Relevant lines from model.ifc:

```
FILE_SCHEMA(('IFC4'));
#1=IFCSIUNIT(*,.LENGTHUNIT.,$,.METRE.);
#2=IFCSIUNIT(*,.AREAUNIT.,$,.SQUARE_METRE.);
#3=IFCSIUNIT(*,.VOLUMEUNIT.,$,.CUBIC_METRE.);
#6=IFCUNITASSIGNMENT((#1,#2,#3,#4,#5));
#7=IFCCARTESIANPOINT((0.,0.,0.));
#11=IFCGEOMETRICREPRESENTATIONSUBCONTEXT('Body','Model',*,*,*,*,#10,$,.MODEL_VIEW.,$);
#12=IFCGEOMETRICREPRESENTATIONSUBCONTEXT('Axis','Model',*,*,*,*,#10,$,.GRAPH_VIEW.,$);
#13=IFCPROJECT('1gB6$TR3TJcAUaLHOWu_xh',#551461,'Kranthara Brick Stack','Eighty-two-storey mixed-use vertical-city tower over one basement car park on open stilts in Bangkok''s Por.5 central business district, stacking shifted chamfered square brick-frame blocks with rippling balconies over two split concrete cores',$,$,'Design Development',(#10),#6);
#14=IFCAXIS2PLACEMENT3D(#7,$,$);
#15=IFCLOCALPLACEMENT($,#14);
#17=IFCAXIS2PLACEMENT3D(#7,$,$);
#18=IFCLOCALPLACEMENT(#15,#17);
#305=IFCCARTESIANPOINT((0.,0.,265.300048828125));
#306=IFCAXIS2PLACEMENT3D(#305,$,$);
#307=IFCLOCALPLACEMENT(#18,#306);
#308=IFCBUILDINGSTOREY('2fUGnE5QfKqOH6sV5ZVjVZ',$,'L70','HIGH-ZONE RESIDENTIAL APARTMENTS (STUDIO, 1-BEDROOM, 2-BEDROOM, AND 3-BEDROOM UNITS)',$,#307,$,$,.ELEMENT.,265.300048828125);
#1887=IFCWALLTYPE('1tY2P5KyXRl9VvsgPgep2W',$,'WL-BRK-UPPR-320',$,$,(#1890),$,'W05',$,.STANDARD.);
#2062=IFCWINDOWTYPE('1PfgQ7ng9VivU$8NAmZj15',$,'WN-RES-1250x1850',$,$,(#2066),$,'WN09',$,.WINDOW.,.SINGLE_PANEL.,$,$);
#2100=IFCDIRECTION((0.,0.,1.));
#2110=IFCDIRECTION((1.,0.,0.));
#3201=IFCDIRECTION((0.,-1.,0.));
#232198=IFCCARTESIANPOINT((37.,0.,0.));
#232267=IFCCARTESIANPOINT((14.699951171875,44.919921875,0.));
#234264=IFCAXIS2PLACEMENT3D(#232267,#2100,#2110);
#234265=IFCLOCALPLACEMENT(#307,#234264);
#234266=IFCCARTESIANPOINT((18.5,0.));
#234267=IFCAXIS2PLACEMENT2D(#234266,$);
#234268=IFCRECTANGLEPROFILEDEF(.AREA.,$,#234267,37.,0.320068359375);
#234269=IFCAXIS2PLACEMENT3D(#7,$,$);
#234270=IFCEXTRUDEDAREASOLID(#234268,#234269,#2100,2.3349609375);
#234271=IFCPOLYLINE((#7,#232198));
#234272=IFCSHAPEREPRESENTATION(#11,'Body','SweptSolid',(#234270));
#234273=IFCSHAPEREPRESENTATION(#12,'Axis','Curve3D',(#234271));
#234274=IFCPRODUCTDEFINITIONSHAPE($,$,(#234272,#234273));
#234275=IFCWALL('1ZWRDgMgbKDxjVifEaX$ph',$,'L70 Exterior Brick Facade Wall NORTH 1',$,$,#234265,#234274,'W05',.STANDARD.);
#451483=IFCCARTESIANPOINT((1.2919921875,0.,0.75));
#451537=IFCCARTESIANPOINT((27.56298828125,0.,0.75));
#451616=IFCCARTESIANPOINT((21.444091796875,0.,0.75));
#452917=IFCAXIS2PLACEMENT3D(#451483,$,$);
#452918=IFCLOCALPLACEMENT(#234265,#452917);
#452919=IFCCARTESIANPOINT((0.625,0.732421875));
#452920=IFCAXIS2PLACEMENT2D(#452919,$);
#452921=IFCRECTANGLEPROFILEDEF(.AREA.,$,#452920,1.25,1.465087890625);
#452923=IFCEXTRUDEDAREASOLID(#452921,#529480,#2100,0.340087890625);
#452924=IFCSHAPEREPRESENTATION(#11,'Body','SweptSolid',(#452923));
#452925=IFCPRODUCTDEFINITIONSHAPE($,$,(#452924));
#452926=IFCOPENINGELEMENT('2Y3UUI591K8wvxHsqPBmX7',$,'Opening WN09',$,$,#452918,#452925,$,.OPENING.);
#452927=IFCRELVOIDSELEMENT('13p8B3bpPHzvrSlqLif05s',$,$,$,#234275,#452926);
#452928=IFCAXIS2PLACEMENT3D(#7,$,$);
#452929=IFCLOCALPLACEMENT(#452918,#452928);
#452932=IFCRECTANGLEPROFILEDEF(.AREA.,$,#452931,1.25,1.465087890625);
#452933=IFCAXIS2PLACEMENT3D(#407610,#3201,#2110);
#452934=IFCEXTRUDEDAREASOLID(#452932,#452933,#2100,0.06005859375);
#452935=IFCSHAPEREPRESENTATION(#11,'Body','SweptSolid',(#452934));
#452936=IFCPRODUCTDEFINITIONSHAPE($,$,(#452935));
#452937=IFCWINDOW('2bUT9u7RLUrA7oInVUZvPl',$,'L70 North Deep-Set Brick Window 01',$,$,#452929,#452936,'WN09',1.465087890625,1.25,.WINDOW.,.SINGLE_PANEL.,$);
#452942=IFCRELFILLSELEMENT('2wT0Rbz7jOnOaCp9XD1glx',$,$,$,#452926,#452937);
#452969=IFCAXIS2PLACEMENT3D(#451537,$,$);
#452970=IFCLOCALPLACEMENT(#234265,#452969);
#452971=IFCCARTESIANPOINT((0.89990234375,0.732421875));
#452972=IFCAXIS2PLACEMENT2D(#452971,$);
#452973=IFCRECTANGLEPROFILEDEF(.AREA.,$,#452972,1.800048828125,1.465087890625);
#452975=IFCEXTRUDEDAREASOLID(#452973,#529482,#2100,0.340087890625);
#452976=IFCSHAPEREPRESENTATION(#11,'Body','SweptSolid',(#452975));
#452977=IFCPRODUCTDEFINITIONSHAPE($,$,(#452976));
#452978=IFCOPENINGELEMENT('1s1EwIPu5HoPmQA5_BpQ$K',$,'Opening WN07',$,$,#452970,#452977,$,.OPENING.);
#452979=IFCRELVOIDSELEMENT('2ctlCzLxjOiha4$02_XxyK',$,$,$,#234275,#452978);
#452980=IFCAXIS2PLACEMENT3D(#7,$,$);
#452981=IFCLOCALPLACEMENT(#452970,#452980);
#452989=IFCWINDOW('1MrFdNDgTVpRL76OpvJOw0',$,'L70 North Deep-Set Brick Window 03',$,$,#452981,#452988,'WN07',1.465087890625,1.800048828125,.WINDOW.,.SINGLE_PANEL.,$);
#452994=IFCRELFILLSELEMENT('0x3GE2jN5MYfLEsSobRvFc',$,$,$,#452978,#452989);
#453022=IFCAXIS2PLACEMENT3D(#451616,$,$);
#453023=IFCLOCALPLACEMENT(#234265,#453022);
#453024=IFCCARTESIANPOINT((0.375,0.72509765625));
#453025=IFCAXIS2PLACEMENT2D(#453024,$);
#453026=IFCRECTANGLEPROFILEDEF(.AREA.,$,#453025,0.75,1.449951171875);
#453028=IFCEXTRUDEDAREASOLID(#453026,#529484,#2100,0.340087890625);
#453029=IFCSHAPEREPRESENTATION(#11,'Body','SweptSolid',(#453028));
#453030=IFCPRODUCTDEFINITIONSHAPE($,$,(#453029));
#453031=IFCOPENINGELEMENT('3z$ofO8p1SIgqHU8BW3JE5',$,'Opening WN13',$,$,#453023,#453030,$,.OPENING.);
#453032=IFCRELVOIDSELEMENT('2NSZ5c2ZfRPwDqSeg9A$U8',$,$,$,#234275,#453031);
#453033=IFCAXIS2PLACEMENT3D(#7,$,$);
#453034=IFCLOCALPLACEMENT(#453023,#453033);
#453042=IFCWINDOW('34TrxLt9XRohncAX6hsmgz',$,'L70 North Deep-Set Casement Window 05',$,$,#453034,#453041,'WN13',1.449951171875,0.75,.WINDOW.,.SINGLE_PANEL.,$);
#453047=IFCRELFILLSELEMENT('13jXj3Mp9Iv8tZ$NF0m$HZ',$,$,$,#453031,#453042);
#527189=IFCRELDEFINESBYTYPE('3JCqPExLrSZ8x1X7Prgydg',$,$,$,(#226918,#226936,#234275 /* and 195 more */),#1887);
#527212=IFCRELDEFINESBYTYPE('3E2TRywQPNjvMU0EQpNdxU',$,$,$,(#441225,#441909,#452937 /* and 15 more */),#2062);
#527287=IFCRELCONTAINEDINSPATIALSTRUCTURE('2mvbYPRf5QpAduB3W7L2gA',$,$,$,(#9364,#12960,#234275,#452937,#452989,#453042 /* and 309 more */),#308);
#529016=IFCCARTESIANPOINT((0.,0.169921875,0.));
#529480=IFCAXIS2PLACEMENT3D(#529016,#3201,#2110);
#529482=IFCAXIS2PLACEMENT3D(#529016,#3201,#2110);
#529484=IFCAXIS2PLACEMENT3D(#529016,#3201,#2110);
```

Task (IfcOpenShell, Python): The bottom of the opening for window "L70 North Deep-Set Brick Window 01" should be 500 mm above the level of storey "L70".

```python
import numpy as np
import ifcopenshell
import ifcopenshell.api.geometry
import ifcopenshell.geom
import ifcopenshell.util.element
import ifcopenshell.util.placement
import ifcopenshell.util.shape
import ifcopenshell.util.unit

model = ifcopenshell.open("model.ifc")
unit_scale = ifcopenshell.util.unit.calculate_unit_scale(model)

window = model.by_guid("2bUT9u7RLUrA7oInVUZvPl")
opening = window.FillsVoids[0].RelatingOpeningElement
storey = ifcopenshell.util.element.get_container(window, ifc_class="IfcBuildingStorey")
level = ifcopenshell.util.placement.get_local_placement(storey.ObjectPlacement)[2, 3]

# The opening's origin need not be at the sill, so measure its lowest point.
shape = ifcopenshell.geom.create_shape(ifcopenshell.geom.settings(), opening)
bottom = ifcopenshell.util.shape.get_shape_bottom_elevation(shape, shape.geometry) / unit_scale
dz = level + 0.5 - bottom

shift = np.array([0.0, 0.0, dz])
# The window is placed relative to its opening, so it follows when the opening moves.
matrix = ifcopenshell.util.placement.get_local_placement(opening.ObjectPlacement)
matrix[:3, 3] += shift
ifcopenshell.api.geometry.edit_object_placement(
    model, product=opening, matrix=matrix, is_si=False, should_transform_children=True
)

print(f"moved by {dz * unit_scale:+.3f} m")

model.write("model_v2.ifc")
```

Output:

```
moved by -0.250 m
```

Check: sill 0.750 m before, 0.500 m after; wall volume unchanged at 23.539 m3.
